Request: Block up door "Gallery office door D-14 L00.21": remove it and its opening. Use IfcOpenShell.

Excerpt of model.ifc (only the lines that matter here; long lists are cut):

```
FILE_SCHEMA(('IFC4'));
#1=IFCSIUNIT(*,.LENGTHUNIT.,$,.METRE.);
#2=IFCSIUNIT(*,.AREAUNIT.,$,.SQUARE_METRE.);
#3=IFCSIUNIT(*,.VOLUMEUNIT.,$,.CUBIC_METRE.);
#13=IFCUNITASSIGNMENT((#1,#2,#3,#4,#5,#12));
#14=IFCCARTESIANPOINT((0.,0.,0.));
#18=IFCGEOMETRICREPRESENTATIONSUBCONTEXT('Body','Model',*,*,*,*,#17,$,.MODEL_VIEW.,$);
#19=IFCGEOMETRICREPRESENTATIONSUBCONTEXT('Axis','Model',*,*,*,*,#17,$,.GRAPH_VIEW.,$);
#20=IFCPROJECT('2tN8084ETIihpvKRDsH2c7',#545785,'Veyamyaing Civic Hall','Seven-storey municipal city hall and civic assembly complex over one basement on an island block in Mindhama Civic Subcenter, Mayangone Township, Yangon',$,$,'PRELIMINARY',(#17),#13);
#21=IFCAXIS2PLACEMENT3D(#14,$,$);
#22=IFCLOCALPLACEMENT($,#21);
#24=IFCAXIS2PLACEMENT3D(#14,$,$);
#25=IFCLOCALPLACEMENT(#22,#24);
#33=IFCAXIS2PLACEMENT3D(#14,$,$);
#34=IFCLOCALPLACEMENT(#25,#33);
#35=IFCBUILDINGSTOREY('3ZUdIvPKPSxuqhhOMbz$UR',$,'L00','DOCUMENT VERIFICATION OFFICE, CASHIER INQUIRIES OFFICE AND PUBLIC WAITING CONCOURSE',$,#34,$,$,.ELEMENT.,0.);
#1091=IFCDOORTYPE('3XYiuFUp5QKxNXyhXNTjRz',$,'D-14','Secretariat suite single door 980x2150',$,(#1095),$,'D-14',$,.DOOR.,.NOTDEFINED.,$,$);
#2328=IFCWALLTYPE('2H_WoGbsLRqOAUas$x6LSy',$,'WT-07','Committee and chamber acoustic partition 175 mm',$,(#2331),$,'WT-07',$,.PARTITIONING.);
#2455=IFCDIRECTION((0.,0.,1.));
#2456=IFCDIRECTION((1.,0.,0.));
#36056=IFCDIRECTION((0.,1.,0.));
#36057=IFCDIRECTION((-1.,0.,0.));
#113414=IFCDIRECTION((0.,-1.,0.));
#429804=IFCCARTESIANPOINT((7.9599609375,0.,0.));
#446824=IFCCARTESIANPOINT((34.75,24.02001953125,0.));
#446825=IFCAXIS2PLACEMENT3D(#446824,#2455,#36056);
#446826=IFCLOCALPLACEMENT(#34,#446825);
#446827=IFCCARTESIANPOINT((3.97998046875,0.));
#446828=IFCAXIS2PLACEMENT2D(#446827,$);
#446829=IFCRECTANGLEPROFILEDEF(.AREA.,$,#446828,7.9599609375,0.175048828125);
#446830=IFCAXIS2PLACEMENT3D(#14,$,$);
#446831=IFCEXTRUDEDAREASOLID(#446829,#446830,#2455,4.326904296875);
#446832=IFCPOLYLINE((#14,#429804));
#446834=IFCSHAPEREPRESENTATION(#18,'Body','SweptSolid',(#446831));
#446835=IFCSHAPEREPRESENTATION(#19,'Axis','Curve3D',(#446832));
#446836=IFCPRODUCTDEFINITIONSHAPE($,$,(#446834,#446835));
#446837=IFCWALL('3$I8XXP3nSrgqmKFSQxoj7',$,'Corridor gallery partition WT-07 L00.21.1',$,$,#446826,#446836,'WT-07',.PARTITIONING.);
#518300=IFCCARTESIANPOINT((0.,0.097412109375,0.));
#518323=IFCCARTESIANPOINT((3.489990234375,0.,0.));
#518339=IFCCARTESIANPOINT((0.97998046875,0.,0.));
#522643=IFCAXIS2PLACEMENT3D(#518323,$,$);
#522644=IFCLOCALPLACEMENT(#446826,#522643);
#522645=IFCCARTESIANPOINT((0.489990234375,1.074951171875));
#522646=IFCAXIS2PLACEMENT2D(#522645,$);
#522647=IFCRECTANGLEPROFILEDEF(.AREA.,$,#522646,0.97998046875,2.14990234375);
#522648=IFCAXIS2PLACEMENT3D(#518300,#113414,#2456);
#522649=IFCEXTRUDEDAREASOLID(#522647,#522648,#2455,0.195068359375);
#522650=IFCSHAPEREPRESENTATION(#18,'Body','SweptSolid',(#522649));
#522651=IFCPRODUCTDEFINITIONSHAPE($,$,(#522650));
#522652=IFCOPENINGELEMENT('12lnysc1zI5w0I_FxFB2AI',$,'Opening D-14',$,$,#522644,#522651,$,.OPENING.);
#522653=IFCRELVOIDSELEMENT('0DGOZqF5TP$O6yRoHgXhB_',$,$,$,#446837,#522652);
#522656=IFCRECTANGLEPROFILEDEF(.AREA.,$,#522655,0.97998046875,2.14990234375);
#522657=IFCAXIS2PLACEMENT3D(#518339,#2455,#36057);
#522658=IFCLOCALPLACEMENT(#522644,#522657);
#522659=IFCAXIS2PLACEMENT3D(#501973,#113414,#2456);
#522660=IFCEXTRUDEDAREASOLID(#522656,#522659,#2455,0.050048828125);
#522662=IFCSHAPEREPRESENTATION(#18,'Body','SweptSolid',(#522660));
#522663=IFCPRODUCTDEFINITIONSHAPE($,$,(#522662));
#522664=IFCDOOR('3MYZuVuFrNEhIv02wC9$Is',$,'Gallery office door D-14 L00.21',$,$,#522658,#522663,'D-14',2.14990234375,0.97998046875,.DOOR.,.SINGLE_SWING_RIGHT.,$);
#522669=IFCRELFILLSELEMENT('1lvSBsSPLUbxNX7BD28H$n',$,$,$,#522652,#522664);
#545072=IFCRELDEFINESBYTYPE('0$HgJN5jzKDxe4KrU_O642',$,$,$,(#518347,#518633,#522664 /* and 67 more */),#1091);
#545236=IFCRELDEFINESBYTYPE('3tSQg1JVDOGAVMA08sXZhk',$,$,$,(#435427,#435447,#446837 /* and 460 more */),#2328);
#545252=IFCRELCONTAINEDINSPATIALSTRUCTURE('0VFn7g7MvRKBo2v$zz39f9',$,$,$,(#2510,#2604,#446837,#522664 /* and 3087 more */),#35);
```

```python
import ifcopenshell
import ifcopenshell.api.feature
import ifcopenshell.api.root
import ifcopenshell.geom
import ifcopenshell.util.shape

model = ifcopenshell.open("model.ifc")
settings = ifcopenshell.geom.settings()


def volume(element):
    """Net volume in cubic metres, openings subtracted."""
    shape = ifcopenshell.geom.create_shape(settings, element)
    return ifcopenshell.util.shape.get_volume(shape.geometry)


door = model.by_guid("3MYZuVuFrNEhIv02wC9$Is")
opening = door.FillsVoids[0].RelatingOpeningElement
wall = opening.VoidsElements[0].RelatingBuildingElement
before = volume(wall)

ifcopenshell.api.root.remove_product(model, product=door)
ifcopenshell.api.feature.remove_feature(model, feature=opening)

after = volume(wall)

print(f"wall volume {before:.3f} -> {after:.3f} m3")

model.write("model_rev.ifc")
```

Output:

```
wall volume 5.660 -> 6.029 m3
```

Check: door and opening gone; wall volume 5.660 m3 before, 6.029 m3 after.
